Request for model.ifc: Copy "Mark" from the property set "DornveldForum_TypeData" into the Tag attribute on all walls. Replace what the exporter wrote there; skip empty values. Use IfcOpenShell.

First a look at what the model holds.

```python
import ifcopenshell
import ifcopenshell.util.element

model = ifcopenshell.open("model.ifc")
print(model.schema)
walls = model.by_type("IfcWall")
print(len(walls), "walls")
for e in walls[:8]:
    source = ifcopenshell.util.element.get_pset(e, "DornveldForum_TypeData", "Mark")
    target = e.Tag
    print(e.id(), repr(source), repr(target), sep=" | ")
```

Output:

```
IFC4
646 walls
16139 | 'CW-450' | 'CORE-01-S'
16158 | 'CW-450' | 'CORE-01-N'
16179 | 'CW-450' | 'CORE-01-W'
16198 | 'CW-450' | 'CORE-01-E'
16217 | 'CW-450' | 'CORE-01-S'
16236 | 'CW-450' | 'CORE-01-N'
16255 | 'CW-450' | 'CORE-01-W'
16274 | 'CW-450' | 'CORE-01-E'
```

```python
import ifcopenshell
import ifcopenshell.util.element

model = ifcopenshell.open("model.ifc")

count = 0
for e in model.by_type("IfcWall"):
    value = ifcopenshell.util.element.get_pset(e, "DornveldForum_TypeData", "Mark")
    current = e.Tag
    if not value or not value.strip() or current == value:
        continue
    e.Tag = value
    count += 1

print(count, "walls updated")

model.write("model_rev.ifc")
```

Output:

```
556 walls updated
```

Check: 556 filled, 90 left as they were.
